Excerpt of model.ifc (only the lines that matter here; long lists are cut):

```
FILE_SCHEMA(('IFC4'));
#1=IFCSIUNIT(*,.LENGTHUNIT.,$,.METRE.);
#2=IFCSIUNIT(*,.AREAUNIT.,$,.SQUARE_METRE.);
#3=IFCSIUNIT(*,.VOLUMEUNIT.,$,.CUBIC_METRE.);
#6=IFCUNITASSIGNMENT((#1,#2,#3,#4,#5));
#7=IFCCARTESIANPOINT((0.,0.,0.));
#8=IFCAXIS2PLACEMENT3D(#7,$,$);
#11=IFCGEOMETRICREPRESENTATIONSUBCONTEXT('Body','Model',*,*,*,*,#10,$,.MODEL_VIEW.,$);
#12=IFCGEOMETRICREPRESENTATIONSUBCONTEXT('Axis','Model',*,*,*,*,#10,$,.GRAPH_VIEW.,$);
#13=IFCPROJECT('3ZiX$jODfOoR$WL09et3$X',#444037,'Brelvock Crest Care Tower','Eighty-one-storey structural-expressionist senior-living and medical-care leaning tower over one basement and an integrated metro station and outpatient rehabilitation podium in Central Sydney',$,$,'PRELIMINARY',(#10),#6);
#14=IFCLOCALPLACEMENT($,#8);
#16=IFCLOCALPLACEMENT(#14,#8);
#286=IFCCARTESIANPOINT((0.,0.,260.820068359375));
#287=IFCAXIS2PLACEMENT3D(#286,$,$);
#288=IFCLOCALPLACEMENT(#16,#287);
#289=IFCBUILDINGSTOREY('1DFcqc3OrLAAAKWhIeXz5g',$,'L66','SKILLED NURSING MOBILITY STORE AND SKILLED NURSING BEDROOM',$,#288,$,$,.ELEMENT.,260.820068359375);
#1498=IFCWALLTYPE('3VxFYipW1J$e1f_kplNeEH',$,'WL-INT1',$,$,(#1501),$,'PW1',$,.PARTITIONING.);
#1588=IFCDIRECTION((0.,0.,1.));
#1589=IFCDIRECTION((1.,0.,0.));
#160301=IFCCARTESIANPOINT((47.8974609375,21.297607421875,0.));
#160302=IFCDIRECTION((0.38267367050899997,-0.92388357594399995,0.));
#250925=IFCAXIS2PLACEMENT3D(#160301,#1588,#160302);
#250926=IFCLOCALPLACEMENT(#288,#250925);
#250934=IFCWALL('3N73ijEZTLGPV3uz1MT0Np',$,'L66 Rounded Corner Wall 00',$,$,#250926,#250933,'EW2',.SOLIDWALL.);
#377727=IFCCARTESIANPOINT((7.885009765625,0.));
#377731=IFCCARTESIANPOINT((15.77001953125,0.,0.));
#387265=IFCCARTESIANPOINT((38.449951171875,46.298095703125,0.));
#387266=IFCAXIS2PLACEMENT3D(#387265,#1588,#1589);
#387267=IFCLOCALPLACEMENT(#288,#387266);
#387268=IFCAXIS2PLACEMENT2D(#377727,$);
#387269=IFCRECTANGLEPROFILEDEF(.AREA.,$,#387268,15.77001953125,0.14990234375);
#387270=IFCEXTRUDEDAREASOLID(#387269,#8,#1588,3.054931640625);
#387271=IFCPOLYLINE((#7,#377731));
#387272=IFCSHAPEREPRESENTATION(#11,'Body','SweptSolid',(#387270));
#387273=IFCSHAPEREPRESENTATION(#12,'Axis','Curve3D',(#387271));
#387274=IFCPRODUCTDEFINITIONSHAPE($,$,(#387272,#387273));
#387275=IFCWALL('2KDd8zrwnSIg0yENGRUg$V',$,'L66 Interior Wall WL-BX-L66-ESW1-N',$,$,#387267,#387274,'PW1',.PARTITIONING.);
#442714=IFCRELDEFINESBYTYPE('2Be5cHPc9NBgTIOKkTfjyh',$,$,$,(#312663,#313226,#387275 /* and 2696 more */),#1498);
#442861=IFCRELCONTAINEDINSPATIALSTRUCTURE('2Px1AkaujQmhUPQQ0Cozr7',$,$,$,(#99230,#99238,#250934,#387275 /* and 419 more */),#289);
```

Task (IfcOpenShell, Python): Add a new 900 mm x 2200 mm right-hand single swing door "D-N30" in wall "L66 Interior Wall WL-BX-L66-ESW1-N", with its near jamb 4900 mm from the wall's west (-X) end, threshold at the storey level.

```python
import numpy as np
import ifcopenshell
import ifcopenshell.api.feature
import ifcopenshell.api.geometry
import ifcopenshell.api.root
import ifcopenshell.api.spatial
import ifcopenshell.geom
import ifcopenshell.util.element
import ifcopenshell.util.placement
import ifcopenshell.util.representation
import ifcopenshell.util.shape
import ifcopenshell.util.unit

model = ifcopenshell.open("model.ifc")
unit_scale = ifcopenshell.util.unit.calculate_unit_scale(model)
settings = ifcopenshell.geom.settings()


def volume(element):
    """Net volume in cubic metres, openings subtracted."""
    shape = ifcopenshell.geom.create_shape(settings, element)
    return ifcopenshell.util.shape.get_volume(shape.geometry)


wall = model.by_guid("2KDd8zrwnSIg0yENGRUg$V")
storey = ifcopenshell.util.element.get_container(wall, ifc_class="IfcBuildingStorey")
context = ifcopenshell.util.representation.get_context(model, "Model", "Body", "MODEL_VIEW")
before = volume(wall)

width, height, from_end, sill = 0.9, 2.2, 4.9, 0.0  # metres

# The wall runs along its own X axis, and the end named is its -X end.
wall_shape = ifcopenshell.geom.create_shape(settings, wall)
x, y, z = ifcopenshell.util.shape.get_vertices(wall_shape.geometry).T
start = x.min() + from_end
face, thickness = float(y.min()), float(y.max() - y.min())
wall_matrix = ifcopenshell.util.placement.get_local_placement(wall.ObjectPlacement)
level = ifcopenshell.util.placement.get_local_placement(storey.ObjectPlacement)[2, 3]


def in_wall(x, y):
    """Placement at x, y metres in the wall's axes, at sill height."""
    matrix = wall_matrix.copy()
    matrix[:, 3] = wall_matrix @ np.array([x / unit_scale, y / unit_scale, 0.0, 1.0])
    matrix[2, 3] = level + sill / unit_scale
    return matrix


# Opening: a box that overshoots both wall faces by 50 mm.
opening = ifcopenshell.api.root.create_entity(model, ifc_class="IfcOpeningElement", predefined_type="OPENING")
box = ifcopenshell.api.geometry.add_wall_representation(
    model, context=context, length=width, height=height, thickness=thickness + 0.1
)
ifcopenshell.api.geometry.assign_representation(model, product=opening, representation=box)
ifcopenshell.api.geometry.edit_object_placement(model, product=opening, matrix=in_wall(start, face - 0.05), is_si=False)
ifcopenshell.api.feature.add_feature(model, feature=opening, element=wall)

door = ifcopenshell.api.root.create_entity(model, ifc_class="IfcDoor", name="D-N30", predefined_type="DOOR")
door.OverallWidth, door.OverallHeight = width / unit_scale, height / unit_scale
door.OperationType = "SINGLE_SWING_RIGHT"
body = ifcopenshell.api.geometry.add_door_representation(
    model,
    context=context,
    overall_width=door.OverallWidth,
    overall_height=door.OverallHeight,
    operation_type="SINGLE_SWING_RIGHT",
    lining_properties={"LiningDepth": thickness / unit_scale, "ThresholdDepth": thickness / unit_scale},
)
ifcopenshell.api.geometry.assign_representation(model, product=door, representation=body)
ifcopenshell.api.spatial.assign_container(model, products=[door], relating_structure=storey)
ifcopenshell.api.feature.add_filling(model, opening=opening, element=door)

# The lining spans the wall, so the door starts at the wall face.
ifcopenshell.api.geometry.edit_object_placement(model, product=door, matrix=in_wall(start, face), is_si=False)

after = volume(wall)

print(f"wall volume {before:.3f} -> {after:.3f} m3")

model.write("model-out.ifc")
```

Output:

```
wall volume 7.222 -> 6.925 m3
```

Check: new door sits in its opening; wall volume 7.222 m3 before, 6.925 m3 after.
